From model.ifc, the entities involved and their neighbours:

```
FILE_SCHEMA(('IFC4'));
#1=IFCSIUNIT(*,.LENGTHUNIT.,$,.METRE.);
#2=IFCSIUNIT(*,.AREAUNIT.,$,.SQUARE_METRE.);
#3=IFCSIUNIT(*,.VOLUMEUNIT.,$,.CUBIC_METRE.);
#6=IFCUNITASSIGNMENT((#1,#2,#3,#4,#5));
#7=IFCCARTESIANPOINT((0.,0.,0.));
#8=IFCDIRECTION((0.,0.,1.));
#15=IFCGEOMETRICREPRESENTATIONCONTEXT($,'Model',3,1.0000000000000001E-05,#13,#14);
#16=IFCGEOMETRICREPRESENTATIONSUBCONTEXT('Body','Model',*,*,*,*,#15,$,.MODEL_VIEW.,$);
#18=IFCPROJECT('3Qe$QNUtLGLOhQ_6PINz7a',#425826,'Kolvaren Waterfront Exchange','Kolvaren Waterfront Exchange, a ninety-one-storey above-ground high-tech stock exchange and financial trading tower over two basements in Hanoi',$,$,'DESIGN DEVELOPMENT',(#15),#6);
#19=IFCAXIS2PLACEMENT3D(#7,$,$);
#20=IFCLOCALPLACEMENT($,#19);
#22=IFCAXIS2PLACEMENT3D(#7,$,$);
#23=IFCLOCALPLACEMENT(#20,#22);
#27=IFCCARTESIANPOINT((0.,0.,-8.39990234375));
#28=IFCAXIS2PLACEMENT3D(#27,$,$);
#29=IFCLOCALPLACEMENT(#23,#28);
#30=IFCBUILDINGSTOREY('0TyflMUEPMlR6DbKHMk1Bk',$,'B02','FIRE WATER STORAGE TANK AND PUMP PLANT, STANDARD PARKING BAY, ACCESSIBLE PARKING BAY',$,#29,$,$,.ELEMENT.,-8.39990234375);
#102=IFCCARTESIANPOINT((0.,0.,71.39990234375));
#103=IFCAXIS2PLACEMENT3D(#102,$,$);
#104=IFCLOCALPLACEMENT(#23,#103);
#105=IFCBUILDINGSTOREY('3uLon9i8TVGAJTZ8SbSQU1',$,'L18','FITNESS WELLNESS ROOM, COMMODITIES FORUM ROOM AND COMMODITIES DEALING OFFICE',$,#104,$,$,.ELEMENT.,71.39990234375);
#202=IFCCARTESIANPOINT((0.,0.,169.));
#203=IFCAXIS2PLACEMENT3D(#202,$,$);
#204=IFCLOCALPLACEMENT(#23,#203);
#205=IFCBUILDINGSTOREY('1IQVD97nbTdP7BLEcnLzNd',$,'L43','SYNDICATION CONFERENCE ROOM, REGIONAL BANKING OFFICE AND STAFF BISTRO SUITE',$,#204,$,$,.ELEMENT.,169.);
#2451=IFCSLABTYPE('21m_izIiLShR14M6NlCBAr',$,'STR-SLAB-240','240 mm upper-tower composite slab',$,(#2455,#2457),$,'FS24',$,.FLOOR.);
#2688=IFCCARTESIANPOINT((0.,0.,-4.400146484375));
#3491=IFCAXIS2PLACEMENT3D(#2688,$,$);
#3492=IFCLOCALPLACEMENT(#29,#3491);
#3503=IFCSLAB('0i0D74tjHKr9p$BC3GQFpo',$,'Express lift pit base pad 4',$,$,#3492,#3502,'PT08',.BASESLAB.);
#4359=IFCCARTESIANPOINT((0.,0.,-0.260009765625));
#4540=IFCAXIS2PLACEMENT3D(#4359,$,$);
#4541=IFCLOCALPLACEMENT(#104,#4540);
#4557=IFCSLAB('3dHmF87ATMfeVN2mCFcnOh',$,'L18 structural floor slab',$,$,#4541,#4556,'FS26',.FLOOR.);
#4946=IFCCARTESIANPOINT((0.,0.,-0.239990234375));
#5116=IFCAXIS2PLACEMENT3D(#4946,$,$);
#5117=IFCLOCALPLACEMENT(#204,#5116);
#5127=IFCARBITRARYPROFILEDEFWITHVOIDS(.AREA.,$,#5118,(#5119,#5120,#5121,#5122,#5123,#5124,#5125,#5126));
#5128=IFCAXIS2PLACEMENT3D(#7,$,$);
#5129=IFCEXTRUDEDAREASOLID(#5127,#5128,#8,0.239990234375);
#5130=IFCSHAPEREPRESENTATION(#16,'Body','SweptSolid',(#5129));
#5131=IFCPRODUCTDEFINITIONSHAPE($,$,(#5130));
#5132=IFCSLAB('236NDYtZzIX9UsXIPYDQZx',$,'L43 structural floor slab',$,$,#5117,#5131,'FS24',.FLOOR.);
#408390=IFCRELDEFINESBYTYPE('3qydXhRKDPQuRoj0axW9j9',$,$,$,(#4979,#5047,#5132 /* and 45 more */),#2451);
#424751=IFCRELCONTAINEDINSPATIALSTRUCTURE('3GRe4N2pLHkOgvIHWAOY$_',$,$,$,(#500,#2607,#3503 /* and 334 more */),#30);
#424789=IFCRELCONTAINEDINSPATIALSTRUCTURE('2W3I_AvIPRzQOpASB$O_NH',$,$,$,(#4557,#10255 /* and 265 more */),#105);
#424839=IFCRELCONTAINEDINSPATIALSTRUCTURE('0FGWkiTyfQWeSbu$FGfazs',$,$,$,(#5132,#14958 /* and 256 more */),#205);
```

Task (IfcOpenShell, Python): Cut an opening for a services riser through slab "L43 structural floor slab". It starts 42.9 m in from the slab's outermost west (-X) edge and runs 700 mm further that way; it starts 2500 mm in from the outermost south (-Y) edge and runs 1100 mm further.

```python
import numpy as np
import ifcopenshell
import ifcopenshell.api.feature
import ifcopenshell.api.geometry
import ifcopenshell.api.root
import ifcopenshell.geom
import ifcopenshell.util.placement
import ifcopenshell.util.representation
import ifcopenshell.util.shape
import ifcopenshell.util.unit

model = ifcopenshell.open("model.ifc")
unit_scale = ifcopenshell.util.unit.calculate_unit_scale(model)
settings = ifcopenshell.geom.settings()


def volume(element):
    """Net volume in cubic metres, openings subtracted."""
    shape = ifcopenshell.geom.create_shape(settings, element)
    return ifcopenshell.util.shape.get_volume(shape.geometry)


slab = model.by_guid("236NDYtZzIX9UsXIPYDQZx")
before = volume(slab)

# Extent in the slab's own axes, in metres. The edges named are its -X and -Y sides.
slab_shape = ifcopenshell.geom.create_shape(settings, slab)
vertices = ifcopenshell.util.shape.get_vertices(slab_shape.geometry)
x_min, y_min, bottom = vertices.min(axis=0)
top = vertices[:, 2].max()

opening = ifcopenshell.api.root.create_entity(model, ifc_class="IfcOpeningElement", name="Services riser opening", predefined_type="OPENING")
context = ifcopenshell.util.representation.get_context(model, "Model", "Body", "MODEL_VIEW")
width, depth = 0.7, 1.1
outline = [(0.0, 0.0), (width, 0.0), (width, depth), (0.0, depth), (0.0, 0.0)]
# Overshoot both faces by 50 mm so the cut is clean.
shape = ifcopenshell.api.geometry.add_slab_representation(
    model, context=context, depth=top - bottom + 0.1, polyline=outline
)
ifcopenshell.api.geometry.assign_representation(model, product=opening, representation=shape)

matrix = ifcopenshell.util.placement.get_local_placement(slab.ObjectPlacement)
matrix[:, 3] = matrix @ np.append(np.array([x_min + 42.9, y_min + 2.5, bottom - 0.05]) / unit_scale, 1.0)
ifcopenshell.api.geometry.edit_object_placement(model, product=opening, matrix=matrix, is_si=False)
ifcopenshell.api.feature.add_feature(model, feature=opening, element=slab)

after = volume(slab)

print(f"slab volume {before:.3f} -> {after:.3f} m3")

model.write("model_rev.ifc")
```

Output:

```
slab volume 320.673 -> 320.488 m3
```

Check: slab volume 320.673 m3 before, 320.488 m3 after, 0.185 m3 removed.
